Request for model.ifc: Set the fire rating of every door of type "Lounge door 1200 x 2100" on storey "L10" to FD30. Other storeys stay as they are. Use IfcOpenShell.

First a look at what the model holds.

```python
import ifcopenshell
import ifcopenshell.util.element

model = ifcopenshell.open("model.ifc")
print(model.schema)
storey = next(s for s in model.by_type("IfcBuildingStorey") if s.Name == "L10")
doors = [e for e in ifcopenshell.util.element.get_decomposition(storey) if e.is_a("IfcDoor")]
seen = {}
for e in doors:
    element_type = ifcopenshell.util.element.get_type(e)
    key = (element_type.Name if element_type != e and element_type else None, ifcopenshell.util.element.get_pset(e, "Pset_DoorCommon", "FireRating"))
    seen[key] = seen.get(key, 0) + 1
for (name, value), count in sorted(seen.items(), key=str):
    print(count, "x", name, "|", value)
```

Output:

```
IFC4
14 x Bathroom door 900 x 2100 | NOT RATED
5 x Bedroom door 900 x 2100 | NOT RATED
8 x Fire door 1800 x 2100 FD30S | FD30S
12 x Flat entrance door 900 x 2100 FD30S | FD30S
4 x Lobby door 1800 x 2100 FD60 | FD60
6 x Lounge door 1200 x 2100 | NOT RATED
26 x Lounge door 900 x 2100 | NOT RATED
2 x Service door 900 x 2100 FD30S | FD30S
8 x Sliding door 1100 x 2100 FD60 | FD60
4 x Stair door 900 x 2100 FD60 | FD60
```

```python
import ifcopenshell
import ifcopenshell.api.pset
import ifcopenshell.util.element

model = ifcopenshell.open("model.ifc")

storey = next(s for s in model.by_type("IfcBuildingStorey") if s.Name == "L10")
doors = [e for e in ifcopenshell.util.element.get_decomposition(storey) if e.is_a("IfcDoor")]

count = 0
for e in doors:
    element_type = ifcopenshell.util.element.get_type(e)
    if element_type in (None, e) or element_type.Name != "Lounge door 1200 x 2100":
        continue
    found = ifcopenshell.util.element.get_pset(e, "Pset_DoorCommon", should_inherit=False)
    if found:
        pset = model.by_id(found["id"])
        if len(ifcopenshell.util.element.get_elements_by_pset(pset)) > 1:
            pset = ifcopenshell.api.pset.unshare_pset(model, products=[e], pset=pset)[0]
    else:
        pset = ifcopenshell.api.pset.add_pset(model, product=e, name="Pset_DoorCommon")
    ifcopenshell.api.pset.edit_pset(model, pset=pset, properties={"FireRating": "FD30"})
    count += 1

print(count, "doors updated")

model.write("model_edited.ifc")
```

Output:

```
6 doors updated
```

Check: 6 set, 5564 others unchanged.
